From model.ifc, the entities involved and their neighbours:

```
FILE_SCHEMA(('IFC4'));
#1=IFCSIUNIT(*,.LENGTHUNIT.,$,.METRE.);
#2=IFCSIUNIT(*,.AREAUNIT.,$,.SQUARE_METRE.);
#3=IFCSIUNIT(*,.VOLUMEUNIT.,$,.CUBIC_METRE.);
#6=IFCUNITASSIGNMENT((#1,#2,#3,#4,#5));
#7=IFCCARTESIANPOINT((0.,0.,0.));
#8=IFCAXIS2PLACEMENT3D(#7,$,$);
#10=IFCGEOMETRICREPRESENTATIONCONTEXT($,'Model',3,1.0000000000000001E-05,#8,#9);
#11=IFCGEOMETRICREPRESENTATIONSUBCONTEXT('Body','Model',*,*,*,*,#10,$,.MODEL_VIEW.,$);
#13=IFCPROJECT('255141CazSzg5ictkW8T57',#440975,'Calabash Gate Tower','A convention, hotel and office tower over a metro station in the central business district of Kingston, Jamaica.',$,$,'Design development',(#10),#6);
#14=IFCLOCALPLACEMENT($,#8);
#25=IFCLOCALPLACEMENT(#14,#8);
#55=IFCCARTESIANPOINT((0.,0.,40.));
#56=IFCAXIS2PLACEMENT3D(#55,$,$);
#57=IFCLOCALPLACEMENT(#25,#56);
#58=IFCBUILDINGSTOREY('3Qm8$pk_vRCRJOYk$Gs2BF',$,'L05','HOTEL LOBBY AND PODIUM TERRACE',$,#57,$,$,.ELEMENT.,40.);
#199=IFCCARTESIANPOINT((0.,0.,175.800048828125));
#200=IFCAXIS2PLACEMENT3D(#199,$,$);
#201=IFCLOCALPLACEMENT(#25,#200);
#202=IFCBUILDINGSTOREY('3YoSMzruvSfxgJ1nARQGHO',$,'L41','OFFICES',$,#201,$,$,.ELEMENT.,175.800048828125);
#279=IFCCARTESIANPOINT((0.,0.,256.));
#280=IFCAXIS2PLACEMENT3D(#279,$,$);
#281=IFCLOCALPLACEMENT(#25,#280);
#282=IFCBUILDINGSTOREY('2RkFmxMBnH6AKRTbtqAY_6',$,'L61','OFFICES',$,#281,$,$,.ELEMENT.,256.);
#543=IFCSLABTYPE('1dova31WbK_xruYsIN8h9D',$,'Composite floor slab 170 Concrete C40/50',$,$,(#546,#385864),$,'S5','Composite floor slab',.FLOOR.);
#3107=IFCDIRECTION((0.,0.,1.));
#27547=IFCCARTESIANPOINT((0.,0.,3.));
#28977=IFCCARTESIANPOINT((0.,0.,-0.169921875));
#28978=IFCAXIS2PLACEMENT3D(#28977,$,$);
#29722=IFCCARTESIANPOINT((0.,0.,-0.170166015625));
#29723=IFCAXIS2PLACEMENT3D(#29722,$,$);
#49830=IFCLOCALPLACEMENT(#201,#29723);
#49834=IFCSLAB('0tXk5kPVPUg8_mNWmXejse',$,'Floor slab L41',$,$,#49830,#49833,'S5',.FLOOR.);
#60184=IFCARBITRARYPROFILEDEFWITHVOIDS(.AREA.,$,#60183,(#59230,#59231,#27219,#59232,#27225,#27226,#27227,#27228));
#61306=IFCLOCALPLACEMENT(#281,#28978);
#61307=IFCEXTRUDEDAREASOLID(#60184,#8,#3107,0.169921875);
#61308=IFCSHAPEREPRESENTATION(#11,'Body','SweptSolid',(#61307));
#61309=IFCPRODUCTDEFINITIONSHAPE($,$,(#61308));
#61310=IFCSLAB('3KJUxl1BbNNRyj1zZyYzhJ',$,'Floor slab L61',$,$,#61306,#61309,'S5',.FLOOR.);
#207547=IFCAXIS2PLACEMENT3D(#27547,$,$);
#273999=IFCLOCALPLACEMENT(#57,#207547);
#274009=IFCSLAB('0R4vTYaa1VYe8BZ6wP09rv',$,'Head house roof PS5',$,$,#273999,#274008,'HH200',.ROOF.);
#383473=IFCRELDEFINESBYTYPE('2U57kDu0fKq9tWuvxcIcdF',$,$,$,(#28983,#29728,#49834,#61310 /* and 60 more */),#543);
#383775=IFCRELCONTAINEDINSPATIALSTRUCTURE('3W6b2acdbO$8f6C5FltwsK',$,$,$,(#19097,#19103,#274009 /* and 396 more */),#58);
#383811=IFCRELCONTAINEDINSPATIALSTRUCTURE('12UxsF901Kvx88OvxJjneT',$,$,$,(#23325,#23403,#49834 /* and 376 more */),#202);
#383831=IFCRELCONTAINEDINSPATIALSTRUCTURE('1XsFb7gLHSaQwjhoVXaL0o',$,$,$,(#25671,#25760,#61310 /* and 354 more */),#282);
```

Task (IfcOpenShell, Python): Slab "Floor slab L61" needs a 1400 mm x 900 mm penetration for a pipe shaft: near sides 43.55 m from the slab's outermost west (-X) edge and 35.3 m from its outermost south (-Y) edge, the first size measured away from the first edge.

```python
import numpy as np
import ifcopenshell
import ifcopenshell.api.feature
import ifcopenshell.api.geometry
import ifcopenshell.api.root
import ifcopenshell.geom
import ifcopenshell.util.placement
import ifcopenshell.util.representation
import ifcopenshell.util.shape
import ifcopenshell.util.unit

model = ifcopenshell.open("model.ifc")
unit_scale = ifcopenshell.util.unit.calculate_unit_scale(model)
settings = ifcopenshell.geom.settings()


def volume(element):
    """Net volume in cubic metres, openings subtracted."""
    shape = ifcopenshell.geom.create_shape(settings, element)
    return ifcopenshell.util.shape.get_volume(shape.geometry)


slab = model.by_id(61310)
before = volume(slab)

# Extent in the slab's own axes, in metres. The edges named are its -X and -Y sides.
slab_shape = ifcopenshell.geom.create_shape(settings, slab)
vertices = ifcopenshell.util.shape.get_vertices(slab_shape.geometry)
x_min, y_min, bottom = vertices.min(axis=0)
top = vertices[:, 2].max()

opening = ifcopenshell.api.root.create_entity(model, ifc_class="IfcOpeningElement", name="Pipe shaft opening", predefined_type="OPENING")
context = ifcopenshell.util.representation.get_context(model, "Model", "Body", "MODEL_VIEW")
width, depth = 1.4, 0.9
outline = [(0.0, 0.0), (width, 0.0), (width, depth), (0.0, depth), (0.0, 0.0)]
# Overshoot both faces by 50 mm so the cut is clean.
shape = ifcopenshell.api.geometry.add_slab_representation(
    model, context=context, depth=top - bottom + 0.1, polyline=outline
)
ifcopenshell.api.geometry.assign_representation(model, product=opening, representation=shape)

matrix = ifcopenshell.util.placement.get_local_placement(slab.ObjectPlacement)
matrix[:, 3] = matrix @ np.append(np.array([x_min + 43.55, y_min + 35.3, bottom - 0.05]) / unit_scale, 1.0)
ifcopenshell.api.geometry.edit_object_placement(model, product=opening, matrix=matrix, is_si=False)
ifcopenshell.api.feature.add_feature(model, feature=opening, element=slab)

after = volume(slab)

print(f"slab volume {before:.3f} -> {after:.3f} m3")

model.write("model_v2.ifc")
```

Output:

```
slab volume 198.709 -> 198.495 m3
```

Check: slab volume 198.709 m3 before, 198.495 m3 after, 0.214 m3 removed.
